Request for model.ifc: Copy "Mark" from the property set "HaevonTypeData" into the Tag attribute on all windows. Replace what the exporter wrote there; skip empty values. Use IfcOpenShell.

First a look at what the model holds.

```python
import ifcopenshell
import ifcopenshell.util.element

model = ifcopenshell.open("model.ifc")
print(model.schema)
windows = model.by_type("IfcWindow")
print(len(windows), "windows")
for e in windows[:8]:
    source = ifcopenshell.util.element.get_pset(e, "HaevonTypeData", "Mark")
    target = e.Tag
    print(e.id(), repr(source), repr(target), sep=" | ")
```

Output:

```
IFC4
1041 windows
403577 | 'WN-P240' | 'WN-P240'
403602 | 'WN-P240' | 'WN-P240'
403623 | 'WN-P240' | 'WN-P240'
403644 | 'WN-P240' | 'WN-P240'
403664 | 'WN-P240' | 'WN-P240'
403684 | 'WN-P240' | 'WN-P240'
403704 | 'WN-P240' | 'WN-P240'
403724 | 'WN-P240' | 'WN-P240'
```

```python
import ifcopenshell
import ifcopenshell.util.element

model = ifcopenshell.open("model.ifc")

count = 0
for e in model.by_type("IfcWindow"):
    value = ifcopenshell.util.element.get_pset(e, "HaevonTypeData", "Mark")
    current = e.Tag
    if not value or not value.strip() or current == value:
        continue
    e.Tag = value
    count += 1

print(count, "windows updated")

model.write("model_rev.ifc")
```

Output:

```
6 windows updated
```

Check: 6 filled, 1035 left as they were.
